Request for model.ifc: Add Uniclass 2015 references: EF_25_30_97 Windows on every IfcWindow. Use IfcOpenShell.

First a look at what the model holds.

```python
import ifcopenshell

model = ifcopenshell.open("model.ifc")
print(model.schema)
print("classifications:", [c.Name for c in model.by_type("IfcClassification")])
for ifc_class in ("IfcDoor", "IfcRoof", "IfcStair", "IfcWall", "IfcWindow"):
    print(ifc_class, len(model.by_type(ifc_class)))
```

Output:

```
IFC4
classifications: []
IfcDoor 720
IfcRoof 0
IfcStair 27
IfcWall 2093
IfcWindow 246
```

```python
import ifcopenshell
import ifcopenshell.api.classification

model = ifcopenshell.open("model.ifc")

system = ifcopenshell.api.classification.add_classification(model, classification="Uniclass 2015")

codes = {
    "IfcWindow": ("EF_25_30_97", "Windows"),
}
for ifc_class, (code, name) in codes.items():
    products = model.by_type(ifc_class)
    ifcopenshell.api.classification.add_reference(
        model, products=products, classification=system, identification=code, name=name
    )
    print(code, len(products))

model.write("model_updated.ifc")
```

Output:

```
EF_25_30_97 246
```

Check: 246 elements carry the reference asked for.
